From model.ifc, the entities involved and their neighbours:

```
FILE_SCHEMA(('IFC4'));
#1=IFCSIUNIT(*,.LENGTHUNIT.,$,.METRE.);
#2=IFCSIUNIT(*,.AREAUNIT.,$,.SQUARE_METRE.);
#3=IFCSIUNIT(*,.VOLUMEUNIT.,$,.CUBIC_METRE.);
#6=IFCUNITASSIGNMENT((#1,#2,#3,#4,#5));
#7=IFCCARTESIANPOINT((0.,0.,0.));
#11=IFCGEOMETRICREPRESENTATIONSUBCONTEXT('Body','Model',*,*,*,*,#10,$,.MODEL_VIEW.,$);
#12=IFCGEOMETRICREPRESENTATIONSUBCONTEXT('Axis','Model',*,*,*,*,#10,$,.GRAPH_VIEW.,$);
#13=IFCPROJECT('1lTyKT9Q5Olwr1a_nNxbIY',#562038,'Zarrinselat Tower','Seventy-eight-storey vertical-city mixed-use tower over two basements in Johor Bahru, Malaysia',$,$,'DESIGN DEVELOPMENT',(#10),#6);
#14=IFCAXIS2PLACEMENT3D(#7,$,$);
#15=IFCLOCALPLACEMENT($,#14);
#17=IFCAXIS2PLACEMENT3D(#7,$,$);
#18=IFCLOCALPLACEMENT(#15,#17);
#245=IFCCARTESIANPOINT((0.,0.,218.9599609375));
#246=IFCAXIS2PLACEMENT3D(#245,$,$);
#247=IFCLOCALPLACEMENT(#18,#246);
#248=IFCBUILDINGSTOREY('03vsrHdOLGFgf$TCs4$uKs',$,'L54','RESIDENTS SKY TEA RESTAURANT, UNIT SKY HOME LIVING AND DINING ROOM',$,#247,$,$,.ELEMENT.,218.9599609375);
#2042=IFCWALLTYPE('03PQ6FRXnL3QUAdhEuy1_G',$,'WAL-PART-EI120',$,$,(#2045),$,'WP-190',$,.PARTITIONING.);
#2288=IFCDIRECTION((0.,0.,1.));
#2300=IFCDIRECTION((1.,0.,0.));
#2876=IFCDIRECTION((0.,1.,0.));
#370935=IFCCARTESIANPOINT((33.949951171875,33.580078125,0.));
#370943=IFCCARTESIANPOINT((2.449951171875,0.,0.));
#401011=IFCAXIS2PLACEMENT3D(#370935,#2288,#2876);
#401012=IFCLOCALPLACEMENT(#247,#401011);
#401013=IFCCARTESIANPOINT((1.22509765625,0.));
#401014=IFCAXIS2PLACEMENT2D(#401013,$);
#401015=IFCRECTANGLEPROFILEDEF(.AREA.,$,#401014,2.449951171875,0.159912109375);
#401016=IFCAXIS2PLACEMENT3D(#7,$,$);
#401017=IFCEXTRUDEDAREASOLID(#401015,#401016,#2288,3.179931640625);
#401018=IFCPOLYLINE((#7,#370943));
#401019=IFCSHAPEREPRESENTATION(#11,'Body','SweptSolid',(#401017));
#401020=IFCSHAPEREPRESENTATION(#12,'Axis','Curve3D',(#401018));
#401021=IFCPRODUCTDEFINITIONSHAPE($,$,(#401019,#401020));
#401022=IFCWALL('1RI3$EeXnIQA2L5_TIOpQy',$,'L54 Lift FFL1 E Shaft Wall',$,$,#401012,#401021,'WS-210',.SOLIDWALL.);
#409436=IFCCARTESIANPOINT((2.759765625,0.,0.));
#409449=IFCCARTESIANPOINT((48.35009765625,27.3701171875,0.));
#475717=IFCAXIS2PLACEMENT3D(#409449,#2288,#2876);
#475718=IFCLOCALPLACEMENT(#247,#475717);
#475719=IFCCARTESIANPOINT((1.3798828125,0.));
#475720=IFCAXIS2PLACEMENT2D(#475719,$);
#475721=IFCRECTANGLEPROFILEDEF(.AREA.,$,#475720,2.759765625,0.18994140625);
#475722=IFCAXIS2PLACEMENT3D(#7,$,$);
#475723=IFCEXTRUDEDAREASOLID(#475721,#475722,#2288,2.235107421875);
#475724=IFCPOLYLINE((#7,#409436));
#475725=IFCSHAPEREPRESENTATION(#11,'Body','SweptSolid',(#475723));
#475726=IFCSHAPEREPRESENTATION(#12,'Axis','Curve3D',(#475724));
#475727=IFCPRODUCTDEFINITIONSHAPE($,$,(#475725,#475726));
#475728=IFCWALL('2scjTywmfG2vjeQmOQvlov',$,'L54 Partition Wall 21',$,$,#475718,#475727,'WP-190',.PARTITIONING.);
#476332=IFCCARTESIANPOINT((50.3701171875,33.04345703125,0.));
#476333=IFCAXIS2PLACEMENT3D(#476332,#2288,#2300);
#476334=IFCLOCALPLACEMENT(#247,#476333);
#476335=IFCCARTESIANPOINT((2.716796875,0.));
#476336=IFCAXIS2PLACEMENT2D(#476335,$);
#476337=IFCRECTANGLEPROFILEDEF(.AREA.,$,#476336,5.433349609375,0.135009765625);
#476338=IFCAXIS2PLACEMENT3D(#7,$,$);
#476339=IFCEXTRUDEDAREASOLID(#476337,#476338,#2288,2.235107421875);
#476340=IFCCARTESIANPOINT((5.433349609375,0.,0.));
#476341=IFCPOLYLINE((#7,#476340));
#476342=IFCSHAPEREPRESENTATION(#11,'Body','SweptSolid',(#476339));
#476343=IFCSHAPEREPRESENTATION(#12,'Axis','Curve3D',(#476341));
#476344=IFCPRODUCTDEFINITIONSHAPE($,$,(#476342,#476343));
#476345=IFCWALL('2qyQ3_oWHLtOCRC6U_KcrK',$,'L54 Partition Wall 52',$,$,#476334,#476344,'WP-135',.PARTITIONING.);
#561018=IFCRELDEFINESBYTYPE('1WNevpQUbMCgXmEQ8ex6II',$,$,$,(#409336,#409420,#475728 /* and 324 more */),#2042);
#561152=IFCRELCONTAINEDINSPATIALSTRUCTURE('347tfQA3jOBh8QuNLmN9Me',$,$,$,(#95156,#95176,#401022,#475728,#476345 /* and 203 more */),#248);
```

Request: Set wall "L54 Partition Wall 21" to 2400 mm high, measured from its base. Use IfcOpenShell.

```python
import ifcopenshell
import ifcopenshell.geom
import ifcopenshell.util.representation
import ifcopenshell.util.shape
import ifcopenshell.util.unit

model = ifcopenshell.open("model.ifc")
unit_scale = ifcopenshell.util.unit.calculate_unit_scale(model)
settings = ifcopenshell.geom.settings()


def volume(element):
    """Net volume in cubic metres, openings subtracted."""
    shape = ifcopenshell.geom.create_shape(settings, element)
    return ifcopenshell.util.shape.get_volume(shape.geometry)


wall = model.by_guid("2scjTywmfG2vjeQmOQvlov")
before = volume(wall)

body = ifcopenshell.util.representation.get_representation(wall, "Model", "Body")
solid = body.Items[0]
old_height = solid.Depth
solid.Depth = 2.4 / unit_scale
after = volume(wall)

print(f"height {old_height:g} -> {solid.Depth:g}, volume {before:.3f} -> {after:.3f} m3")

model.write("model_rev.ifc")
```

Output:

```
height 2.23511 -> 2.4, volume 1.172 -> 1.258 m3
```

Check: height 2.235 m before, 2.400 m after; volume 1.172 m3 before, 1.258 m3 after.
